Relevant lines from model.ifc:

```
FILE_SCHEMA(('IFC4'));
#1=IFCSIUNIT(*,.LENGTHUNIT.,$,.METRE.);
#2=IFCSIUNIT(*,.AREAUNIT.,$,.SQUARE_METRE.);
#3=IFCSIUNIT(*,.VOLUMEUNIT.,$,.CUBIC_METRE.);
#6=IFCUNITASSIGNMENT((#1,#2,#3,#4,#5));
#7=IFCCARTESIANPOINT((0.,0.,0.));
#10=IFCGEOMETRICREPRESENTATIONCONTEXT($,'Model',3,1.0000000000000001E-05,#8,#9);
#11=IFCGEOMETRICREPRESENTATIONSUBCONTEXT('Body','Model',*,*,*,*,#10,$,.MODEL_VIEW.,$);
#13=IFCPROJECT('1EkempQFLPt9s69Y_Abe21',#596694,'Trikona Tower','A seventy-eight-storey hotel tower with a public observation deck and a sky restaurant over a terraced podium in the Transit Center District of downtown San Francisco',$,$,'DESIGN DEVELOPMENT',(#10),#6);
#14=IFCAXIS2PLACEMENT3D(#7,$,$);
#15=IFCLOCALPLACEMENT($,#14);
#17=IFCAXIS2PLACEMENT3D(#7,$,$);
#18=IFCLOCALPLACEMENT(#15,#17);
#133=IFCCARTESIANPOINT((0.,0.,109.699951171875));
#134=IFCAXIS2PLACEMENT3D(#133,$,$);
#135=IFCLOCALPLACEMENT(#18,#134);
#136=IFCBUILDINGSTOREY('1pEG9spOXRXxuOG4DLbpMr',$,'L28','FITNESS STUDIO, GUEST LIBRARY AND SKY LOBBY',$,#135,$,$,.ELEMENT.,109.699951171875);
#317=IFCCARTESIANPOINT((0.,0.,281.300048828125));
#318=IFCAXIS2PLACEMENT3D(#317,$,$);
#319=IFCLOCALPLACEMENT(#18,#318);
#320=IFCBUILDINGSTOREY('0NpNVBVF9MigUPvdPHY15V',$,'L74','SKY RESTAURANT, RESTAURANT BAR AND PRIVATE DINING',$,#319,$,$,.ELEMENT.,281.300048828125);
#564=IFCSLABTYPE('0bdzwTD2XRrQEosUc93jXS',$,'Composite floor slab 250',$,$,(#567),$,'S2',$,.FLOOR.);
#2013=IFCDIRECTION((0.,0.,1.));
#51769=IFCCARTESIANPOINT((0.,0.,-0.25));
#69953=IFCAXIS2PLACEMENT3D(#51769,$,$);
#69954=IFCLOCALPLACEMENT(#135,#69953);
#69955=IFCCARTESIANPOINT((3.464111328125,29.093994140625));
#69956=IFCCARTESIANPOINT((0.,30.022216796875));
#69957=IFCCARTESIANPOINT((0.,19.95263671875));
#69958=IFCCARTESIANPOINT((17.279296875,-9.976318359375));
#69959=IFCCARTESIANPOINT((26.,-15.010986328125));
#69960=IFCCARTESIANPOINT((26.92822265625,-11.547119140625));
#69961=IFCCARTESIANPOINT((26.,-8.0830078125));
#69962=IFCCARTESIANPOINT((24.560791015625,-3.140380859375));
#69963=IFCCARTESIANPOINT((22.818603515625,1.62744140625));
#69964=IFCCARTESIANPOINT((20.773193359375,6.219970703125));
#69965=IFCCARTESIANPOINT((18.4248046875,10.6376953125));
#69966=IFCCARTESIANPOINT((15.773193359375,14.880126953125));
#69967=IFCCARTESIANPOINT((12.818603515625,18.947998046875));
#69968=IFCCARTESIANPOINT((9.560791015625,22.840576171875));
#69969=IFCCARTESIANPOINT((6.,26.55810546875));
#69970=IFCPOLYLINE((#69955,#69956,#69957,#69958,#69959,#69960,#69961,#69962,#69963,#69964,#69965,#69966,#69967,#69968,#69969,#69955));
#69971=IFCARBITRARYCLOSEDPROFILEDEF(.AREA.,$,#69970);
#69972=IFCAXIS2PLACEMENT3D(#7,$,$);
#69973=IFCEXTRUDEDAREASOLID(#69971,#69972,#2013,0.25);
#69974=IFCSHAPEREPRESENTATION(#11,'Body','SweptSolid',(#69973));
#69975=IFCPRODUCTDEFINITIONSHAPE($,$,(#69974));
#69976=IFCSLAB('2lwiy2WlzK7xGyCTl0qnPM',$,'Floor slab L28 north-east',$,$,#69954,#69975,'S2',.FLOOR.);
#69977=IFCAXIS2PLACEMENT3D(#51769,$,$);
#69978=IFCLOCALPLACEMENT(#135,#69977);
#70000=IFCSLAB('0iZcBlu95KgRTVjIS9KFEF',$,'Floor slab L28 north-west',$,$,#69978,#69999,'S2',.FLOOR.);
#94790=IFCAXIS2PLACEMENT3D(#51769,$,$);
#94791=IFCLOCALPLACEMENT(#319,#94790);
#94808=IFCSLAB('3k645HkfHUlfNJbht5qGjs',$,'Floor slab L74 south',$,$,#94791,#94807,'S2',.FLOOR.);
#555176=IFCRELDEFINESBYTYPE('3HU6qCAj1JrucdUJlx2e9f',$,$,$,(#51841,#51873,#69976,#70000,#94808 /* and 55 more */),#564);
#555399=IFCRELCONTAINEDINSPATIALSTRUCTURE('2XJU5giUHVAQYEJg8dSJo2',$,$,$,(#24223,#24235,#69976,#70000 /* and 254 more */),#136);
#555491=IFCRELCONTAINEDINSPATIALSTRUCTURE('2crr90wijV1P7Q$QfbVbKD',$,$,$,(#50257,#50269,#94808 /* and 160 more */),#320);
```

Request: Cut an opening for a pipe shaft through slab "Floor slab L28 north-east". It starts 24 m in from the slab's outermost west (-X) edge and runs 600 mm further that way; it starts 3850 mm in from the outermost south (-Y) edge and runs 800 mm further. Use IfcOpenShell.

```python
import numpy as np
import ifcopenshell
import ifcopenshell.api.feature
import ifcopenshell.api.geometry
import ifcopenshell.api.root
import ifcopenshell.geom
import ifcopenshell.util.placement
import ifcopenshell.util.representation
import ifcopenshell.util.shape
import ifcopenshell.util.unit

model = ifcopenshell.open("model.ifc")
unit_scale = ifcopenshell.util.unit.calculate_unit_scale(model)
settings = ifcopenshell.geom.settings()


def volume(element):
    """Net volume in cubic metres, openings subtracted."""
    shape = ifcopenshell.geom.create_shape(settings, element)
    return ifcopenshell.util.shape.get_volume(shape.geometry)


slab = model.by_guid("2lwiy2WlzK7xGyCTl0qnPM")
before = volume(slab)

# Extent in the slab's own axes, in metres. The edges named are its -X and -Y sides.
slab_shape = ifcopenshell.geom.create_shape(settings, slab)
vertices = ifcopenshell.util.shape.get_vertices(slab_shape.geometry)
x_min, y_min, bottom = vertices.min(axis=0)
top = vertices[:, 2].max()

opening = ifcopenshell.api.root.create_entity(model, ifc_class="IfcOpeningElement", name="Pipe shaft opening", predefined_type="OPENING")
context = ifcopenshell.util.representation.get_context(model, "Model", "Body", "MODEL_VIEW")
width, depth = 0.6, 0.8
outline = [(0.0, 0.0), (width, 0.0), (width, depth), (0.0, depth), (0.0, 0.0)]
# Overshoot both faces by 50 mm so the cut is clean.
shape = ifcopenshell.api.geometry.add_slab_representation(
    model, context=context, depth=top - bottom + 0.1, polyline=outline
)
ifcopenshell.api.geometry.assign_representation(model, product=opening, representation=shape)

matrix = ifcopenshell.util.placement.get_local_placement(slab.ObjectPlacement)
matrix[:, 3] = matrix @ np.append(np.array([x_min + 24, y_min + 3.85, bottom - 0.05]) / unit_scale, 1.0)
ifcopenshell.api.geometry.edit_object_placement(model, product=opening, matrix=matrix, is_si=False)
ifcopenshell.api.feature.add_feature(model, feature=opening, element=slab)

after = volume(slab)

print(f"slab volume {before:.3f} -> {after:.3f} m3")

model.write("model_edited.ifc")
```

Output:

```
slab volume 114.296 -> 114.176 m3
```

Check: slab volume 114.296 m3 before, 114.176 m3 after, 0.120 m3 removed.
